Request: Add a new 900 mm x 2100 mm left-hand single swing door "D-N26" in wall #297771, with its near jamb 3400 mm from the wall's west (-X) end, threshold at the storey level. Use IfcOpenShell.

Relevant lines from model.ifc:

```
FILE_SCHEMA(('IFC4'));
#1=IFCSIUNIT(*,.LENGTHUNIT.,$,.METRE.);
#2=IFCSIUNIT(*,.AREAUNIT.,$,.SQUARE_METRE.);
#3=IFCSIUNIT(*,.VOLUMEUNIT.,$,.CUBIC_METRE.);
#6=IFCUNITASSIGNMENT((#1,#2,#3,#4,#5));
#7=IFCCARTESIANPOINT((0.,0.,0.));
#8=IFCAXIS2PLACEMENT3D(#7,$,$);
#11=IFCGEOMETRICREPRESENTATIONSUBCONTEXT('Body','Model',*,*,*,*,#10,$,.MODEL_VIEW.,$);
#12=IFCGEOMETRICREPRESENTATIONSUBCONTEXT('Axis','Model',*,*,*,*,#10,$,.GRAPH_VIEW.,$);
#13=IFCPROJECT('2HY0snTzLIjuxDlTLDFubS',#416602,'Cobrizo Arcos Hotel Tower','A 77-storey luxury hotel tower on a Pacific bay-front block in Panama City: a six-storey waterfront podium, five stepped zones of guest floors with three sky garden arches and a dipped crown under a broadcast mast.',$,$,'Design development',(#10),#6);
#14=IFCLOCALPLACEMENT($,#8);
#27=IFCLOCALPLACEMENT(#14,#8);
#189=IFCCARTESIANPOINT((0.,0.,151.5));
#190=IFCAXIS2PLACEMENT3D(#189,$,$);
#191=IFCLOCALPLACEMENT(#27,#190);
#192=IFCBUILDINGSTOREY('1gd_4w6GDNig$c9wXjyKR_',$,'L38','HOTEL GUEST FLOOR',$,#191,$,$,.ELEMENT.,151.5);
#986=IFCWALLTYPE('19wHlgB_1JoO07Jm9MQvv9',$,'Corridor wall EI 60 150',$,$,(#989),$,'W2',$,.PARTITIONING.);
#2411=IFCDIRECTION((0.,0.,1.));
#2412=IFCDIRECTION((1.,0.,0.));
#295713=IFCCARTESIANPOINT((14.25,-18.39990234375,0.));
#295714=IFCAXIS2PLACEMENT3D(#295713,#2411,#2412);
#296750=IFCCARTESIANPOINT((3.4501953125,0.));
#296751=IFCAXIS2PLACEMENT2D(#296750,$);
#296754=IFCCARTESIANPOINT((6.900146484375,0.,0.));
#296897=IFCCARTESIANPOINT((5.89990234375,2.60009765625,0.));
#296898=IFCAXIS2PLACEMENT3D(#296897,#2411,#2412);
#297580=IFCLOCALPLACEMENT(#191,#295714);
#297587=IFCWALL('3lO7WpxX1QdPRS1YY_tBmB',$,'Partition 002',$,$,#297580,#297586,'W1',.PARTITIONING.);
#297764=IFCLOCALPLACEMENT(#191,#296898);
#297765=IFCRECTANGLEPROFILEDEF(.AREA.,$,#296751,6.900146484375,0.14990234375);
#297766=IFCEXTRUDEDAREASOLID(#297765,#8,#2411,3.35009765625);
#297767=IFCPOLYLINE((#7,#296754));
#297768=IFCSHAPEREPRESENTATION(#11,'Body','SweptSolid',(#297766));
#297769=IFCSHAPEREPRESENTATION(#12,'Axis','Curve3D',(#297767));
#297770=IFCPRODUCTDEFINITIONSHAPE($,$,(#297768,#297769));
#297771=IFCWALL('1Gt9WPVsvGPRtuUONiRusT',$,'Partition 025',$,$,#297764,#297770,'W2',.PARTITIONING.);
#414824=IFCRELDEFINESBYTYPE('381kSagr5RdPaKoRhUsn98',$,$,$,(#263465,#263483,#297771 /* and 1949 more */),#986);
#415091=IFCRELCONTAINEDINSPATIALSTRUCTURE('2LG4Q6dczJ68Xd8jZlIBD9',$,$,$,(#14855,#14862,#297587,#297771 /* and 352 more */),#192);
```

```python
import numpy as np
import ifcopenshell
import ifcopenshell.api.feature
import ifcopenshell.api.geometry
import ifcopenshell.api.root
import ifcopenshell.api.spatial
import ifcopenshell.geom
import ifcopenshell.util.element
import ifcopenshell.util.placement
import ifcopenshell.util.representation
import ifcopenshell.util.shape
import ifcopenshell.util.unit

model = ifcopenshell.open("model.ifc")
unit_scale = ifcopenshell.util.unit.calculate_unit_scale(model)
settings = ifcopenshell.geom.settings()


def volume(element):
    """Net volume in cubic metres, openings subtracted."""
    shape = ifcopenshell.geom.create_shape(settings, element)
    return ifcopenshell.util.shape.get_volume(shape.geometry)


wall = model.by_guid("1Gt9WPVsvGPRtuUONiRusT")
storey = ifcopenshell.util.element.get_container(wall, ifc_class="IfcBuildingStorey")
context = ifcopenshell.util.representation.get_context(model, "Model", "Body", "MODEL_VIEW")
before = volume(wall)

width, height, from_end, sill = 0.9, 2.1, 3.4, 0.0  # metres

# The wall runs along its own X axis, and the end named is its -X end.
wall_shape = ifcopenshell.geom.create_shape(settings, wall)
x, y, z = ifcopenshell.util.shape.get_vertices(wall_shape.geometry).T
start = x.min() + from_end
face, thickness = float(y.min()), float(y.max() - y.min())
wall_matrix = ifcopenshell.util.placement.get_local_placement(wall.ObjectPlacement)
level = ifcopenshell.util.placement.get_local_placement(storey.ObjectPlacement)[2, 3]


def in_wall(x, y):
    """Placement at x, y metres in the wall's axes, at sill height."""
    matrix = wall_matrix.copy()
    matrix[:, 3] = wall_matrix @ np.array([x / unit_scale, y / unit_scale, 0.0, 1.0])
    matrix[2, 3] = level + sill / unit_scale
    return matrix


# Opening: a box that overshoots both wall faces by 50 mm.
opening = ifcopenshell.api.root.create_entity(model, ifc_class="IfcOpeningElement", predefined_type="OPENING")
box = ifcopenshell.api.geometry.add_wall_representation(
    model, context=context, length=width, height=height, thickness=thickness + 0.1
)
ifcopenshell.api.geometry.assign_representation(model, product=opening, representation=box)
ifcopenshell.api.geometry.edit_object_placement(model, product=opening, matrix=in_wall(start, face - 0.05), is_si=False)
ifcopenshell.api.feature.add_feature(model, feature=opening, element=wall)

door = ifcopenshell.api.root.create_entity(model, ifc_class="IfcDoor", name="D-N26", predefined_type="DOOR")
door.OverallWidth, door.OverallHeight = width / unit_scale, height / unit_scale
door.OperationType = "SINGLE_SWING_LEFT"
body = ifcopenshell.api.geometry.add_door_representation(
    model,
    context=context,
    overall_width=door.OverallWidth,
    overall_height=door.OverallHeight,
    operation_type="SINGLE_SWING_LEFT",
    lining_properties={"LiningDepth": thickness / unit_scale, "ThresholdDepth": thickness / unit_scale},
)
ifcopenshell.api.geometry.assign_representation(model, product=door, representation=body)
ifcopenshell.api.spatial.assign_container(model, products=[door], relating_structure=storey)
ifcopenshell.api.feature.add_filling(model, opening=opening, element=door)

# The lining spans the wall, so the door starts at the wall face.
ifcopenshell.api.geometry.edit_object_placement(model, product=door, matrix=in_wall(start, face), is_si=False)

after = volume(wall)

print(f"wall volume {before:.3f} -> {after:.3f} m3")

model.write("model_updated.ifc")
```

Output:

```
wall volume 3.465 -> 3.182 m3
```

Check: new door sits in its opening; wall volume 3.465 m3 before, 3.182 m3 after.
